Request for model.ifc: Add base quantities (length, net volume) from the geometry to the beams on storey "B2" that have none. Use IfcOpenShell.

First a look at what the model holds.

```python
import ifcopenshell
import ifcopenshell.util.element
import ifcopenshell.util.unit

model = ifcopenshell.open("model.ifc")
print(model.schema)
for unit_type in ("LENGTHUNIT", "AREAUNIT", "VOLUMEUNIT"):
    print(unit_type, ifcopenshell.util.unit.calculate_unit_scale(model, unit_type))
storey = next(s for s in model.by_type("IfcBuildingStorey") if s.Name == "B2")
beams = [e for e in ifcopenshell.util.element.get_decomposition(storey) if e.is_a("IfcBeam")]
for e in sorted(beams, key=lambda e: e.id()):
    print(e.id(), e.is_a(), e.Name, list(ifcopenshell.util.element.get_psets(e, qtos_only=True)), sep=" | ")
```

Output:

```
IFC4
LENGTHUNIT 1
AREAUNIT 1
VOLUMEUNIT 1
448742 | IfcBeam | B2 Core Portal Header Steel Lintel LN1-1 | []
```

```python
import ifcopenshell
import ifcopenshell.api.pset
import ifcopenshell.geom
import ifcopenshell.util.element
import ifcopenshell.util.shape
import ifcopenshell.util.unit

model = ifcopenshell.open("model.ifc")
unit_scale = ifcopenshell.util.unit.calculate_unit_scale(model)
volume_scale = ifcopenshell.util.unit.calculate_unit_scale(model, "VOLUMEUNIT")
settings = ifcopenshell.geom.settings()

storey = next(s for s in model.by_type("IfcBuildingStorey") if s.Name == "B2")
beams = [e for e in ifcopenshell.util.element.get_decomposition(storey) if e.is_a("IfcBeam")]

for e in sorted(beams, key=lambda e: e.id()):
    if ifcopenshell.util.element.get_psets(e, qtos_only=True, should_inherit=False):
        continue
    # Geometry comes back in metres, in the element's own axes.
    shape = ifcopenshell.geom.create_shape(settings, e)
    values = {
        "Length": ifcopenshell.util.shape.get_max_xyz(shape.geometry) / unit_scale,
        "NetVolume": ifcopenshell.util.shape.get_volume(shape.geometry) / volume_scale,
    }
    qto = ifcopenshell.api.pset.add_qto(model, product=e, name="Qto_BeamBaseQuantities")
    ifcopenshell.api.pset.edit_qto(model, qto=qto, properties=values)
    print(e.id(), {k: round(v, 3) for k, v in values.items()})

model.write("model_rev.ifc")
```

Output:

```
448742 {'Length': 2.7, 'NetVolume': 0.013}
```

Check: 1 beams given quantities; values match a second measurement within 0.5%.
